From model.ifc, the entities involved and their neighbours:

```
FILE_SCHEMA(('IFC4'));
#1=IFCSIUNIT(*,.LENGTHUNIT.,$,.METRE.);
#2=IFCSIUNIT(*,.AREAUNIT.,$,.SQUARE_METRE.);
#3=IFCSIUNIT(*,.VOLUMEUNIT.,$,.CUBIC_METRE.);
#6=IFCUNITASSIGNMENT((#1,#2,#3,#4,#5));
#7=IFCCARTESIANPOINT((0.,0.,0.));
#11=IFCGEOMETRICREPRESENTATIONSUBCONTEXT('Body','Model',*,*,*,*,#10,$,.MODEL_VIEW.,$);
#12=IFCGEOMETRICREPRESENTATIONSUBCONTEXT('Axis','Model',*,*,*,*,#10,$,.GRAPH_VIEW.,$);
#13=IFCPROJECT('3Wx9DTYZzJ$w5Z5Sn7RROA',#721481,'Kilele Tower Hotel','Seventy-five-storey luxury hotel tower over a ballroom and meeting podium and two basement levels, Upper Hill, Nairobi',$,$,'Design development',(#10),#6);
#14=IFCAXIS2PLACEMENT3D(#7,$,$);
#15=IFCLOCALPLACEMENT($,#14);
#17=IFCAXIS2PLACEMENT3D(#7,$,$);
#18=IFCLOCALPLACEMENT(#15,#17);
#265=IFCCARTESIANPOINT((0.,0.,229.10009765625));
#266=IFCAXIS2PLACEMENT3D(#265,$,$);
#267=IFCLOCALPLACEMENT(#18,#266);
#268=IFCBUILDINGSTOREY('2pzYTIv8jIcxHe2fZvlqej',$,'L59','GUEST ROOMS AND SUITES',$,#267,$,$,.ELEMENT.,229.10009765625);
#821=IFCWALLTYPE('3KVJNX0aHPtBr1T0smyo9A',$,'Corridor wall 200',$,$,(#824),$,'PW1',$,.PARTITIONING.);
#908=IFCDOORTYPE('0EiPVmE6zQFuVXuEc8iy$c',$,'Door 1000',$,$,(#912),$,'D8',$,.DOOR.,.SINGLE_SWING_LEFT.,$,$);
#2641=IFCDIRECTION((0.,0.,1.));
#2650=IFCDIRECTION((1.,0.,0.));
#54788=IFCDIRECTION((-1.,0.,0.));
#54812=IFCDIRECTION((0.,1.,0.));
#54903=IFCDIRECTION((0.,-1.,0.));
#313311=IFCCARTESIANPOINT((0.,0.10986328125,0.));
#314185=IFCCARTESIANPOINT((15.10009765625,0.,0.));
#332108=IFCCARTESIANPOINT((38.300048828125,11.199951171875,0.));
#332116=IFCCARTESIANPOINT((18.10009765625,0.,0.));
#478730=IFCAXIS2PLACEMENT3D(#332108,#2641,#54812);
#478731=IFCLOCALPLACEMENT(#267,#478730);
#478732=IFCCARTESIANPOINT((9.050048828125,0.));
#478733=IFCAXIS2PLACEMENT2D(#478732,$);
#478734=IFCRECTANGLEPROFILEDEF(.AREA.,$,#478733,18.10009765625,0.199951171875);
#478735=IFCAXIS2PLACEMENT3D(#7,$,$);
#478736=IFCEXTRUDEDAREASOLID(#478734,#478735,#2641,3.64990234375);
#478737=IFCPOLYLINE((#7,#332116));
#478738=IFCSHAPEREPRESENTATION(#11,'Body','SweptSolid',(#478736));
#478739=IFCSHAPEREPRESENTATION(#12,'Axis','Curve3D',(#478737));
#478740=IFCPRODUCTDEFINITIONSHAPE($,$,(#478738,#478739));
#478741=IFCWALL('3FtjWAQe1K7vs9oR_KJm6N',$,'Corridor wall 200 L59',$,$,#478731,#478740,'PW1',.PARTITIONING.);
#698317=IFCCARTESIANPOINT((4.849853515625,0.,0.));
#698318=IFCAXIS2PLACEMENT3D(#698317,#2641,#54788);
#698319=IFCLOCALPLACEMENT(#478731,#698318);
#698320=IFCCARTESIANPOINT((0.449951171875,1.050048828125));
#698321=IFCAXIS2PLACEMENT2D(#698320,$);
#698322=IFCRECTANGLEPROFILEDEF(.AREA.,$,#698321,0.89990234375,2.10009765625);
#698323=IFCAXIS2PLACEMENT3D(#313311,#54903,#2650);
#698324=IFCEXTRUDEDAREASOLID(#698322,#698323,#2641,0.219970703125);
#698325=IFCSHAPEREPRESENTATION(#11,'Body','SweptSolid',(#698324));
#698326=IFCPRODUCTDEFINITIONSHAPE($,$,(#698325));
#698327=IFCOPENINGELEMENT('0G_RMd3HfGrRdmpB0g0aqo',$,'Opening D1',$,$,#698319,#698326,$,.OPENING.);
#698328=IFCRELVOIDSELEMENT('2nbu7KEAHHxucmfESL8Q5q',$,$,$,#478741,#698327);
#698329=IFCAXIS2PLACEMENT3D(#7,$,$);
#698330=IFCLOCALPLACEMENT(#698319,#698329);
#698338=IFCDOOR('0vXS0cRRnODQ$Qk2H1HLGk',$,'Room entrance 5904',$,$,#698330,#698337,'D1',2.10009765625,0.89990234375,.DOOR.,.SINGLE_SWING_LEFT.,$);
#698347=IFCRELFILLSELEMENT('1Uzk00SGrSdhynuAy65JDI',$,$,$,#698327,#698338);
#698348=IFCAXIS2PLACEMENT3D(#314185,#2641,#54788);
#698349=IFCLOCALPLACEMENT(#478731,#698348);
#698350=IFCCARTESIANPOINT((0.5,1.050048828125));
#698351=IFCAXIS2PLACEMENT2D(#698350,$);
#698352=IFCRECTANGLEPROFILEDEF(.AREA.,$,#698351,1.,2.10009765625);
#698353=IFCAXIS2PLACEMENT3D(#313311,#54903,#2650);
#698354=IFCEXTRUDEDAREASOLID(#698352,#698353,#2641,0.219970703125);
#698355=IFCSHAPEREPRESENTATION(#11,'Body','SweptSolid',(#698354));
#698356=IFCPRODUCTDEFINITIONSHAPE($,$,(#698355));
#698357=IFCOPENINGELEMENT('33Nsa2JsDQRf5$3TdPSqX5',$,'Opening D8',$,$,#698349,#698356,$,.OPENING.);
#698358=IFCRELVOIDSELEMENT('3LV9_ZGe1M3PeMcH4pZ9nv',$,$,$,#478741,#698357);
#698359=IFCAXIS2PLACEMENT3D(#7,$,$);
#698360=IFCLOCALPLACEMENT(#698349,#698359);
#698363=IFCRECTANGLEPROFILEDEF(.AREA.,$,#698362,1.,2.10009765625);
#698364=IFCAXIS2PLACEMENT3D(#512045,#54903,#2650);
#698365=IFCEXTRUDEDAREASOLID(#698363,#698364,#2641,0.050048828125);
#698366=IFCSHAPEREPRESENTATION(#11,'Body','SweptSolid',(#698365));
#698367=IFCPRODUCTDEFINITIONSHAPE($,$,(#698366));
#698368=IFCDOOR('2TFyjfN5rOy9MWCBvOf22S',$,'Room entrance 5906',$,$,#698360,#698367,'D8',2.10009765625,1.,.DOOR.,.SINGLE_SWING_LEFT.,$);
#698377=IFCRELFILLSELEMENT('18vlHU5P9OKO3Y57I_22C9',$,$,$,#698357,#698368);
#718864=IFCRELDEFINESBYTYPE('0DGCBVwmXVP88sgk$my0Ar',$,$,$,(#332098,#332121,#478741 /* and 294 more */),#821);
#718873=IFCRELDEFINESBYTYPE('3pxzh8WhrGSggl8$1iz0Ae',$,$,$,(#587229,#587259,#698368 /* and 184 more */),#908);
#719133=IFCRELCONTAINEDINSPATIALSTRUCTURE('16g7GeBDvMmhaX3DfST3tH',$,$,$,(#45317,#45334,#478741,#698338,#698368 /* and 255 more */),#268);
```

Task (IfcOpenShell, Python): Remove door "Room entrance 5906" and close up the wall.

```python
import ifcopenshell
import ifcopenshell.api.feature
import ifcopenshell.api.root
import ifcopenshell.geom
import ifcopenshell.util.shape

model = ifcopenshell.open("model.ifc")
settings = ifcopenshell.geom.settings()


def volume(element):
    """Net volume in cubic metres, openings subtracted."""
    shape = ifcopenshell.geom.create_shape(settings, element)
    return ifcopenshell.util.shape.get_volume(shape.geometry)


door = model.by_guid("2TFyjfN5rOy9MWCBvOf22S")
opening = door.FillsVoids[0].RelatingOpeningElement
wall = opening.VoidsElements[0].RelatingBuildingElement
before = volume(wall)

ifcopenshell.api.root.remove_product(model, product=door)
ifcopenshell.api.feature.remove_feature(model, feature=opening)

after = volume(wall)

print(f"wall volume {before:.3f} -> {after:.3f} m3")

model.write("model-out.ifc")
```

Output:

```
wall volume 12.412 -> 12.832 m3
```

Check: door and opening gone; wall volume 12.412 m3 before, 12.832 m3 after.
